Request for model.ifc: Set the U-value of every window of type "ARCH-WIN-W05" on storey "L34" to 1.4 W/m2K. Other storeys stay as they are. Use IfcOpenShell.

First a look at what the model holds.

```python
import ifcopenshell
import ifcopenshell.util.element

model = ifcopenshell.open("model.ifc")
print(model.schema)
storey = next(s for s in model.by_type("IfcBuildingStorey") if s.Name == "L34")
windows = [e for e in ifcopenshell.util.element.get_decomposition(storey) if e.is_a("IfcWindow")]
seen = {}
for e in windows:
    element_type = ifcopenshell.util.element.get_type(e)
    key = (element_type.Name if element_type != e and element_type else None, ifcopenshell.util.element.get_pset(e, "Pset_WindowCommon", "ThermalTransmittance"))
    seen[key] = seen.get(key, 0) + 1
for (name, value), count in sorted(seen.items(), key=str):
    print(count, "x", name, "|", value)
```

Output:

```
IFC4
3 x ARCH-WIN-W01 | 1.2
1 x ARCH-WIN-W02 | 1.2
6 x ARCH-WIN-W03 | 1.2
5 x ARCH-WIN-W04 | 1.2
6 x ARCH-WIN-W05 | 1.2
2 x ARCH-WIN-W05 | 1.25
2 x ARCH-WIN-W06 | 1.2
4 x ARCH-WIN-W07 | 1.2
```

```python
import ifcopenshell
import ifcopenshell.api.pset
import ifcopenshell.util.element

model = ifcopenshell.open("model.ifc")

storey = next(s for s in model.by_type("IfcBuildingStorey") if s.Name == "L34")
windows = [e for e in ifcopenshell.util.element.get_decomposition(storey) if e.is_a("IfcWindow")]

count = 0
for e in windows:
    element_type = ifcopenshell.util.element.get_type(e)
    if element_type in (None, e) or element_type.Name != "ARCH-WIN-W05":
        continue
    found = ifcopenshell.util.element.get_pset(e, "Pset_WindowCommon", should_inherit=False)
    if found:
        pset = model.by_id(found["id"])
        if len(ifcopenshell.util.element.get_elements_by_pset(pset)) > 1:
            pset = ifcopenshell.api.pset.unshare_pset(model, products=[e], pset=pset)[0]
    else:
        pset = ifcopenshell.api.pset.add_pset(model, product=e, name="Pset_WindowCommon")
    ifcopenshell.api.pset.edit_pset(model, pset=pset, properties={"ThermalTransmittance": 1.4})
    count += 1

print(count, "windows updated")

model.write("model-out.ifc")
```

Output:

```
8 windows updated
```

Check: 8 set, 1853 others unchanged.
